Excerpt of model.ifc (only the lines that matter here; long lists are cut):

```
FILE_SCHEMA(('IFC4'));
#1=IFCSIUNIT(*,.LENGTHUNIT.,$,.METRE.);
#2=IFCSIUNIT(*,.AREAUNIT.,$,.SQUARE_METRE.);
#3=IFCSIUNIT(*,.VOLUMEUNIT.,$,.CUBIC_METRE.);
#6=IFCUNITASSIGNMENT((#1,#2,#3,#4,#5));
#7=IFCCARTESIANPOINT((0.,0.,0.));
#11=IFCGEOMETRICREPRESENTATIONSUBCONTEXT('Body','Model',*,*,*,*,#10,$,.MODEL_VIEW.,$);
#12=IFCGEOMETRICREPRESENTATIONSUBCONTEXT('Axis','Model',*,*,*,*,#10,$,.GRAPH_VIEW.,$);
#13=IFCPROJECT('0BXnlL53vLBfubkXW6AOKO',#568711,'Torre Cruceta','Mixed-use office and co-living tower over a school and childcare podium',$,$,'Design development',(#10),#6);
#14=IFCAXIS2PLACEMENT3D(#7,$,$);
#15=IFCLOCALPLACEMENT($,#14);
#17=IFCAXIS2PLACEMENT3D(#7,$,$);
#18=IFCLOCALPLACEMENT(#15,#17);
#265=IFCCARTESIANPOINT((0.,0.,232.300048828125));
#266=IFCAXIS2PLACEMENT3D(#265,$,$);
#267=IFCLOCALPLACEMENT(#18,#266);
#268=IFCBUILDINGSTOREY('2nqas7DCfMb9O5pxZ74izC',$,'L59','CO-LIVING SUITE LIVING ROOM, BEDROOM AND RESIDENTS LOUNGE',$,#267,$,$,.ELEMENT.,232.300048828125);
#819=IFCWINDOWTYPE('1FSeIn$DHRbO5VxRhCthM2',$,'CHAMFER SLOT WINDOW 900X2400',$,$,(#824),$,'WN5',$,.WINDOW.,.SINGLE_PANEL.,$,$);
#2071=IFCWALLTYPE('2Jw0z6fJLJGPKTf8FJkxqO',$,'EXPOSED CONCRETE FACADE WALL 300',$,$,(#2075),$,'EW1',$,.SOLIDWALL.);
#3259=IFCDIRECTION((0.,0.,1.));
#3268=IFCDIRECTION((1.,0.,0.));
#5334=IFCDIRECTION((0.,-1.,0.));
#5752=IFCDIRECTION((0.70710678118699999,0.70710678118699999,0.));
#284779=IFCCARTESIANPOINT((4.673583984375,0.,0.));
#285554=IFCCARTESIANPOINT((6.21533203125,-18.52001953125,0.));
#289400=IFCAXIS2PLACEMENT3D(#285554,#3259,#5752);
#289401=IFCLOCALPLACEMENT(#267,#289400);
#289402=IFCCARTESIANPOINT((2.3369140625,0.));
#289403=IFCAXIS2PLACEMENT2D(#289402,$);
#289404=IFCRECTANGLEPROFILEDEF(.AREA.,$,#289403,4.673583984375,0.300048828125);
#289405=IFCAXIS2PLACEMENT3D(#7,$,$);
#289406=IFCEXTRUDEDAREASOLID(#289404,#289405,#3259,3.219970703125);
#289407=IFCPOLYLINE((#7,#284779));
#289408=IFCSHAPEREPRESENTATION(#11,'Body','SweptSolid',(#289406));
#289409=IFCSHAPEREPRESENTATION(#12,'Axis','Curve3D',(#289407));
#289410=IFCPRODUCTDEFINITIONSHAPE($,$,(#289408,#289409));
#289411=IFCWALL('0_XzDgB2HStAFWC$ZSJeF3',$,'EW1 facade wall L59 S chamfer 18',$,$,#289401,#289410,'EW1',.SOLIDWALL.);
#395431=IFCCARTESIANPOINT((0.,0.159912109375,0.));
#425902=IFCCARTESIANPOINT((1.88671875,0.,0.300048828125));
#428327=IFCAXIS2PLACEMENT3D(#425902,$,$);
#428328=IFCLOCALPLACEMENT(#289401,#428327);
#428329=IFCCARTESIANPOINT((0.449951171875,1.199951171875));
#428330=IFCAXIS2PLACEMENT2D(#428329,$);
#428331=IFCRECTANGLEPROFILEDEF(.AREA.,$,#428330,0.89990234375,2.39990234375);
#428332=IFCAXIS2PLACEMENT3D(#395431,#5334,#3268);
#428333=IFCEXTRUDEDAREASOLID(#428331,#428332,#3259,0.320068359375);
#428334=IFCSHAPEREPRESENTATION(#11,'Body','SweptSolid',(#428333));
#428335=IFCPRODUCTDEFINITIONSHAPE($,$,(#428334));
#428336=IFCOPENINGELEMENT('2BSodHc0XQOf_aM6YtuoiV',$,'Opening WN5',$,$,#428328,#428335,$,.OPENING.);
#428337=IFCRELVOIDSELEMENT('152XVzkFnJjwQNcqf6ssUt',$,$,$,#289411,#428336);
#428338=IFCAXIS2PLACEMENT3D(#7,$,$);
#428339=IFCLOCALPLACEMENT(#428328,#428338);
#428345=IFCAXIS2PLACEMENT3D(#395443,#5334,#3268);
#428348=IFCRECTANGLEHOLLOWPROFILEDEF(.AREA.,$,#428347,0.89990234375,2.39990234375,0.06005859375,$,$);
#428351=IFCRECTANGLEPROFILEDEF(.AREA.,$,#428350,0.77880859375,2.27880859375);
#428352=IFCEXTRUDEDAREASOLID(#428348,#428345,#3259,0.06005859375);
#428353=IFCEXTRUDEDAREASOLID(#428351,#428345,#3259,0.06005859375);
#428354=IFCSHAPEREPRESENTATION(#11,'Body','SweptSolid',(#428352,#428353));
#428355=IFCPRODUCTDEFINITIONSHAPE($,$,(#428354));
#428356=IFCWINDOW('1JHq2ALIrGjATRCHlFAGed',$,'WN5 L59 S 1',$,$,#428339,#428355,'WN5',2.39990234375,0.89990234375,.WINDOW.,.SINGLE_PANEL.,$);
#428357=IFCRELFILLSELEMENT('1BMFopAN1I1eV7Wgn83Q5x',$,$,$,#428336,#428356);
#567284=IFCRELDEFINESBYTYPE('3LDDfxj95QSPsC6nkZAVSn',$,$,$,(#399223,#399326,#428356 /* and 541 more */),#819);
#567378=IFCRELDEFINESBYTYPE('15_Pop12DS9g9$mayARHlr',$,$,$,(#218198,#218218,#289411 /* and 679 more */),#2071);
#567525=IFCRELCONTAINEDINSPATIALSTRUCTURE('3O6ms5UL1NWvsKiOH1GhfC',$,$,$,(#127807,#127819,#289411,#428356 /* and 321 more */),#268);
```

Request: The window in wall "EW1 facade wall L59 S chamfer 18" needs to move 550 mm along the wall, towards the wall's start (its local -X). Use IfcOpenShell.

```python
import ifcopenshell
import ifcopenshell.api.geometry
import ifcopenshell.util.placement

model = ifcopenshell.open("model.ifc")

window = model.by_guid("1JHq2ALIrGjATRCHlFAGed")
opening = window.FillsVoids[0].RelatingOpeningElement
wall = opening.VoidsElements[0].RelatingBuildingElement

wall_matrix = ifcopenshell.util.placement.get_local_placement(wall.ObjectPlacement)
shift = wall_matrix[:3, 0] * -0.55
before = ifcopenshell.util.placement.get_local_placement(window.ObjectPlacement)[:3, 3].copy()

# The window is placed relative to its opening, so it follows when the opening moves.
matrix = ifcopenshell.util.placement.get_local_placement(opening.ObjectPlacement)
matrix[:3, 3] += shift
ifcopenshell.api.geometry.edit_object_placement(
    model, product=opening, matrix=matrix, is_si=False, should_transform_children=True
)

after = ifcopenshell.util.placement.get_local_placement(window.ObjectPlacement)[:3, 3]
print("window moved by", (after - before).round(3) + 0.0)

model.write("model_updated.ifc")
```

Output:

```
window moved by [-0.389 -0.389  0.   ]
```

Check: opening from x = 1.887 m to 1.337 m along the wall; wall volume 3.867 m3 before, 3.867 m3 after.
